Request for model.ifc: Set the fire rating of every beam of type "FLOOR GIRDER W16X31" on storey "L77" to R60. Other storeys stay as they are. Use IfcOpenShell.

First a look at what the model holds.

```python
import ifcopenshell
import ifcopenshell.util.element

model = ifcopenshell.open("model.ifc")
print(model.schema)
storey = next(s for s in model.by_type("IfcBuildingStorey") if s.Name == "L77")
beams = [e for e in ifcopenshell.util.element.get_decomposition(storey) if e.is_a("IfcBeam")]
seen = {}
for e in beams:
    element_type = ifcopenshell.util.element.get_type(e)
    key = (element_type.Name if element_type != e and element_type else None, ifcopenshell.util.element.get_pset(e, "Pset_BeamCommon", "FireRating"))
    seen[key] = seen.get(key, 0) + 1
for (name, value), count in sorted(seen.items(), key=str):
    print(count, "x", name, "|", value)
```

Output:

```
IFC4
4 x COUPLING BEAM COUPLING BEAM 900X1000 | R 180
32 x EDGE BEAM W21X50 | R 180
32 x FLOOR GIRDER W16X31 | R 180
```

```python
import ifcopenshell
import ifcopenshell.api.pset
import ifcopenshell.util.element

model = ifcopenshell.open("model.ifc")

storey = next(s for s in model.by_type("IfcBuildingStorey") if s.Name == "L77")
beams = [e for e in ifcopenshell.util.element.get_decomposition(storey) if e.is_a("IfcBeam")]

count = 0
for e in beams:
    element_type = ifcopenshell.util.element.get_type(e)
    if element_type in (None, e) or element_type.Name != "FLOOR GIRDER W16X31":
        continue
    found = ifcopenshell.util.element.get_pset(e, "Pset_BeamCommon", should_inherit=False)
    if found:
        pset = model.by_id(found["id"])
        if len(ifcopenshell.util.element.get_elements_by_pset(pset)) > 1:
            pset = ifcopenshell.api.pset.unshare_pset(model, products=[e], pset=pset)[0]
    else:
        pset = ifcopenshell.api.pset.add_pset(model, product=e, name="Pset_BeamCommon")
    ifcopenshell.api.pset.edit_pset(model, pset=pset, properties={"FireRating": "R60"})
    count += 1

print(count, "beams updated")

model.write("model_rev.ifc")
```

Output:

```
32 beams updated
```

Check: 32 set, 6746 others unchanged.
